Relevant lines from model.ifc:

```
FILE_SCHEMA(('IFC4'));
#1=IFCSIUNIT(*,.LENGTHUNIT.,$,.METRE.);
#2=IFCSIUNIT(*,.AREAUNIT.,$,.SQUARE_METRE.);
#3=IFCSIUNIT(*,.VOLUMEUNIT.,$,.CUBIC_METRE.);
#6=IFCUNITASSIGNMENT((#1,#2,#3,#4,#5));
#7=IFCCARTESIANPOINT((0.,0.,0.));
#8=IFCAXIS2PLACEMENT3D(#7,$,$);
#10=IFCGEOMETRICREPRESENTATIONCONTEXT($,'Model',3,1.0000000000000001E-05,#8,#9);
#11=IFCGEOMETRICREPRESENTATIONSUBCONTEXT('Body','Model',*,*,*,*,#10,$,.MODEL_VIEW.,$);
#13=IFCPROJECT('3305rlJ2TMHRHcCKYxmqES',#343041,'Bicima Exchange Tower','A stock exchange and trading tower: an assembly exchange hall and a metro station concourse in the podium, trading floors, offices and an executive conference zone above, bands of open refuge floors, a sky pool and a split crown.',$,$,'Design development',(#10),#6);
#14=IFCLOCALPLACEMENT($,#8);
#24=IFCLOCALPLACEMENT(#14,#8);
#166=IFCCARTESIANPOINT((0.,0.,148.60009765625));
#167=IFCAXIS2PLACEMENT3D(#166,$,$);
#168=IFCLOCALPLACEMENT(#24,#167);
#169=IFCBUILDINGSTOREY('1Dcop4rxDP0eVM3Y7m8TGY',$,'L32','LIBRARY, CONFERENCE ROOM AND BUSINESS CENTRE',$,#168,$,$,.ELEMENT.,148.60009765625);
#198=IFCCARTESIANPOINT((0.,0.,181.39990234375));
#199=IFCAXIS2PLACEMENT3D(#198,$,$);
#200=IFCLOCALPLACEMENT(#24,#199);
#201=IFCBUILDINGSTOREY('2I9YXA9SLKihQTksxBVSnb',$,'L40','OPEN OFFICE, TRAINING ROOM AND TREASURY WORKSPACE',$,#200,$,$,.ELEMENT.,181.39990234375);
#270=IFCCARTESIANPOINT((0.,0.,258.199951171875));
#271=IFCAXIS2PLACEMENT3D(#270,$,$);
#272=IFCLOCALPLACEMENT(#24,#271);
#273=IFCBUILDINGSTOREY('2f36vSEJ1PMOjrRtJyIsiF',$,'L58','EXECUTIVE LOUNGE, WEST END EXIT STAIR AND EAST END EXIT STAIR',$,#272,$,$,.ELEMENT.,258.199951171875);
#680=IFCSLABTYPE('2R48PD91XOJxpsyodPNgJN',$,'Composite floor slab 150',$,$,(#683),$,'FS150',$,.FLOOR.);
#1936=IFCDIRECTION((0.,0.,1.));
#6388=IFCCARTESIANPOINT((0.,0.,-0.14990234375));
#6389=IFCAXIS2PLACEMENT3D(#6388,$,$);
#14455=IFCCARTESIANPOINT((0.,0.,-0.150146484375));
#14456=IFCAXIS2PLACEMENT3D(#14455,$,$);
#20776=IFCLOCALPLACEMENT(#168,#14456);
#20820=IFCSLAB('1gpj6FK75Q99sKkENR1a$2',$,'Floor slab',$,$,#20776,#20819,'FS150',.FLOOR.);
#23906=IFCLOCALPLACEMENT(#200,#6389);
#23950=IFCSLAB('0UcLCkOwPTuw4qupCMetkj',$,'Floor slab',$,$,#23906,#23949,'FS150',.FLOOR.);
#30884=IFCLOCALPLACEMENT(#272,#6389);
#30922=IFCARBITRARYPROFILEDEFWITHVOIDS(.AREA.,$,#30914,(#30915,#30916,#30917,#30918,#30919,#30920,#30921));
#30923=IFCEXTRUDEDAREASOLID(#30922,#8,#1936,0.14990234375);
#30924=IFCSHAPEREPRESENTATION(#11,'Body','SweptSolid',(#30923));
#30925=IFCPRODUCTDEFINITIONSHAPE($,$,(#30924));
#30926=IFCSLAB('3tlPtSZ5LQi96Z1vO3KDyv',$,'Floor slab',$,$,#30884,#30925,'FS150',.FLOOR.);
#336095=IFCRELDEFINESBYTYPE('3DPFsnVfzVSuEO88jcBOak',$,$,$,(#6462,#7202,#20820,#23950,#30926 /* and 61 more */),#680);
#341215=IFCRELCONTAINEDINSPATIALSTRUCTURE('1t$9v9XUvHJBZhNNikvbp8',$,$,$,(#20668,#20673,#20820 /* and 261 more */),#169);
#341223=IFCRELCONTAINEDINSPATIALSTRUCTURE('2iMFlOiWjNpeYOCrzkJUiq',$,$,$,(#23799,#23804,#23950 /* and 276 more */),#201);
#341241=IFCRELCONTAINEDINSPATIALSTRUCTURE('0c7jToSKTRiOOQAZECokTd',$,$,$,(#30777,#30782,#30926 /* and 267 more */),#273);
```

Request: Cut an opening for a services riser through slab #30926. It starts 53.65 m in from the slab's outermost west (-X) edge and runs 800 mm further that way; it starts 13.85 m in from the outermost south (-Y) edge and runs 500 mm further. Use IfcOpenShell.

```python
import numpy as np
import ifcopenshell
import ifcopenshell.api.feature
import ifcopenshell.api.geometry
import ifcopenshell.api.root
import ifcopenshell.geom
import ifcopenshell.util.placement
import ifcopenshell.util.representation
import ifcopenshell.util.shape
import ifcopenshell.util.unit

model = ifcopenshell.open("model.ifc")
unit_scale = ifcopenshell.util.unit.calculate_unit_scale(model)
settings = ifcopenshell.geom.settings()


def volume(element):
    """Net volume in cubic metres, openings subtracted."""
    shape = ifcopenshell.geom.create_shape(settings, element)
    return ifcopenshell.util.shape.get_volume(shape.geometry)


slab = model.by_guid("3tlPtSZ5LQi96Z1vO3KDyv")
before = volume(slab)

# Extent in the slab's own axes, in metres. The edges named are its -X and -Y sides.
slab_shape = ifcopenshell.geom.create_shape(settings, slab)
vertices = ifcopenshell.util.shape.get_vertices(slab_shape.geometry)
x_min, y_min, bottom = vertices.min(axis=0)
top = vertices[:, 2].max()

opening = ifcopenshell.api.root.create_entity(model, ifc_class="IfcOpeningElement", name="Services riser opening", predefined_type="OPENING")
context = ifcopenshell.util.representation.get_context(model, "Model", "Body", "MODEL_VIEW")
width, depth = 0.8, 0.5
outline = [(0.0, 0.0), (width, 0.0), (width, depth), (0.0, depth), (0.0, 0.0)]
# Overshoot both faces by 50 mm so the cut is clean.
shape = ifcopenshell.api.geometry.add_slab_representation(
    model, context=context, depth=top - bottom + 0.1, polyline=outline
)
ifcopenshell.api.geometry.assign_representation(model, product=opening, representation=shape)

matrix = ifcopenshell.util.placement.get_local_placement(slab.ObjectPlacement)
matrix[:, 3] = matrix @ np.append(np.array([x_min + 53.65, y_min + 13.85, bottom - 0.05]) / unit_scale, 1.0)
ifcopenshell.api.geometry.edit_object_placement(model, product=opening, matrix=matrix, is_si=False)
ifcopenshell.api.feature.add_feature(model, feature=opening, element=slab)

after = volume(slab)

print(f"slab volume {before:.3f} -> {after:.3f} m3")

model.write("model_updated.ifc")
```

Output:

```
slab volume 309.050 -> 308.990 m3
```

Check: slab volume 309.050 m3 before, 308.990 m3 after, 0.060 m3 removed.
